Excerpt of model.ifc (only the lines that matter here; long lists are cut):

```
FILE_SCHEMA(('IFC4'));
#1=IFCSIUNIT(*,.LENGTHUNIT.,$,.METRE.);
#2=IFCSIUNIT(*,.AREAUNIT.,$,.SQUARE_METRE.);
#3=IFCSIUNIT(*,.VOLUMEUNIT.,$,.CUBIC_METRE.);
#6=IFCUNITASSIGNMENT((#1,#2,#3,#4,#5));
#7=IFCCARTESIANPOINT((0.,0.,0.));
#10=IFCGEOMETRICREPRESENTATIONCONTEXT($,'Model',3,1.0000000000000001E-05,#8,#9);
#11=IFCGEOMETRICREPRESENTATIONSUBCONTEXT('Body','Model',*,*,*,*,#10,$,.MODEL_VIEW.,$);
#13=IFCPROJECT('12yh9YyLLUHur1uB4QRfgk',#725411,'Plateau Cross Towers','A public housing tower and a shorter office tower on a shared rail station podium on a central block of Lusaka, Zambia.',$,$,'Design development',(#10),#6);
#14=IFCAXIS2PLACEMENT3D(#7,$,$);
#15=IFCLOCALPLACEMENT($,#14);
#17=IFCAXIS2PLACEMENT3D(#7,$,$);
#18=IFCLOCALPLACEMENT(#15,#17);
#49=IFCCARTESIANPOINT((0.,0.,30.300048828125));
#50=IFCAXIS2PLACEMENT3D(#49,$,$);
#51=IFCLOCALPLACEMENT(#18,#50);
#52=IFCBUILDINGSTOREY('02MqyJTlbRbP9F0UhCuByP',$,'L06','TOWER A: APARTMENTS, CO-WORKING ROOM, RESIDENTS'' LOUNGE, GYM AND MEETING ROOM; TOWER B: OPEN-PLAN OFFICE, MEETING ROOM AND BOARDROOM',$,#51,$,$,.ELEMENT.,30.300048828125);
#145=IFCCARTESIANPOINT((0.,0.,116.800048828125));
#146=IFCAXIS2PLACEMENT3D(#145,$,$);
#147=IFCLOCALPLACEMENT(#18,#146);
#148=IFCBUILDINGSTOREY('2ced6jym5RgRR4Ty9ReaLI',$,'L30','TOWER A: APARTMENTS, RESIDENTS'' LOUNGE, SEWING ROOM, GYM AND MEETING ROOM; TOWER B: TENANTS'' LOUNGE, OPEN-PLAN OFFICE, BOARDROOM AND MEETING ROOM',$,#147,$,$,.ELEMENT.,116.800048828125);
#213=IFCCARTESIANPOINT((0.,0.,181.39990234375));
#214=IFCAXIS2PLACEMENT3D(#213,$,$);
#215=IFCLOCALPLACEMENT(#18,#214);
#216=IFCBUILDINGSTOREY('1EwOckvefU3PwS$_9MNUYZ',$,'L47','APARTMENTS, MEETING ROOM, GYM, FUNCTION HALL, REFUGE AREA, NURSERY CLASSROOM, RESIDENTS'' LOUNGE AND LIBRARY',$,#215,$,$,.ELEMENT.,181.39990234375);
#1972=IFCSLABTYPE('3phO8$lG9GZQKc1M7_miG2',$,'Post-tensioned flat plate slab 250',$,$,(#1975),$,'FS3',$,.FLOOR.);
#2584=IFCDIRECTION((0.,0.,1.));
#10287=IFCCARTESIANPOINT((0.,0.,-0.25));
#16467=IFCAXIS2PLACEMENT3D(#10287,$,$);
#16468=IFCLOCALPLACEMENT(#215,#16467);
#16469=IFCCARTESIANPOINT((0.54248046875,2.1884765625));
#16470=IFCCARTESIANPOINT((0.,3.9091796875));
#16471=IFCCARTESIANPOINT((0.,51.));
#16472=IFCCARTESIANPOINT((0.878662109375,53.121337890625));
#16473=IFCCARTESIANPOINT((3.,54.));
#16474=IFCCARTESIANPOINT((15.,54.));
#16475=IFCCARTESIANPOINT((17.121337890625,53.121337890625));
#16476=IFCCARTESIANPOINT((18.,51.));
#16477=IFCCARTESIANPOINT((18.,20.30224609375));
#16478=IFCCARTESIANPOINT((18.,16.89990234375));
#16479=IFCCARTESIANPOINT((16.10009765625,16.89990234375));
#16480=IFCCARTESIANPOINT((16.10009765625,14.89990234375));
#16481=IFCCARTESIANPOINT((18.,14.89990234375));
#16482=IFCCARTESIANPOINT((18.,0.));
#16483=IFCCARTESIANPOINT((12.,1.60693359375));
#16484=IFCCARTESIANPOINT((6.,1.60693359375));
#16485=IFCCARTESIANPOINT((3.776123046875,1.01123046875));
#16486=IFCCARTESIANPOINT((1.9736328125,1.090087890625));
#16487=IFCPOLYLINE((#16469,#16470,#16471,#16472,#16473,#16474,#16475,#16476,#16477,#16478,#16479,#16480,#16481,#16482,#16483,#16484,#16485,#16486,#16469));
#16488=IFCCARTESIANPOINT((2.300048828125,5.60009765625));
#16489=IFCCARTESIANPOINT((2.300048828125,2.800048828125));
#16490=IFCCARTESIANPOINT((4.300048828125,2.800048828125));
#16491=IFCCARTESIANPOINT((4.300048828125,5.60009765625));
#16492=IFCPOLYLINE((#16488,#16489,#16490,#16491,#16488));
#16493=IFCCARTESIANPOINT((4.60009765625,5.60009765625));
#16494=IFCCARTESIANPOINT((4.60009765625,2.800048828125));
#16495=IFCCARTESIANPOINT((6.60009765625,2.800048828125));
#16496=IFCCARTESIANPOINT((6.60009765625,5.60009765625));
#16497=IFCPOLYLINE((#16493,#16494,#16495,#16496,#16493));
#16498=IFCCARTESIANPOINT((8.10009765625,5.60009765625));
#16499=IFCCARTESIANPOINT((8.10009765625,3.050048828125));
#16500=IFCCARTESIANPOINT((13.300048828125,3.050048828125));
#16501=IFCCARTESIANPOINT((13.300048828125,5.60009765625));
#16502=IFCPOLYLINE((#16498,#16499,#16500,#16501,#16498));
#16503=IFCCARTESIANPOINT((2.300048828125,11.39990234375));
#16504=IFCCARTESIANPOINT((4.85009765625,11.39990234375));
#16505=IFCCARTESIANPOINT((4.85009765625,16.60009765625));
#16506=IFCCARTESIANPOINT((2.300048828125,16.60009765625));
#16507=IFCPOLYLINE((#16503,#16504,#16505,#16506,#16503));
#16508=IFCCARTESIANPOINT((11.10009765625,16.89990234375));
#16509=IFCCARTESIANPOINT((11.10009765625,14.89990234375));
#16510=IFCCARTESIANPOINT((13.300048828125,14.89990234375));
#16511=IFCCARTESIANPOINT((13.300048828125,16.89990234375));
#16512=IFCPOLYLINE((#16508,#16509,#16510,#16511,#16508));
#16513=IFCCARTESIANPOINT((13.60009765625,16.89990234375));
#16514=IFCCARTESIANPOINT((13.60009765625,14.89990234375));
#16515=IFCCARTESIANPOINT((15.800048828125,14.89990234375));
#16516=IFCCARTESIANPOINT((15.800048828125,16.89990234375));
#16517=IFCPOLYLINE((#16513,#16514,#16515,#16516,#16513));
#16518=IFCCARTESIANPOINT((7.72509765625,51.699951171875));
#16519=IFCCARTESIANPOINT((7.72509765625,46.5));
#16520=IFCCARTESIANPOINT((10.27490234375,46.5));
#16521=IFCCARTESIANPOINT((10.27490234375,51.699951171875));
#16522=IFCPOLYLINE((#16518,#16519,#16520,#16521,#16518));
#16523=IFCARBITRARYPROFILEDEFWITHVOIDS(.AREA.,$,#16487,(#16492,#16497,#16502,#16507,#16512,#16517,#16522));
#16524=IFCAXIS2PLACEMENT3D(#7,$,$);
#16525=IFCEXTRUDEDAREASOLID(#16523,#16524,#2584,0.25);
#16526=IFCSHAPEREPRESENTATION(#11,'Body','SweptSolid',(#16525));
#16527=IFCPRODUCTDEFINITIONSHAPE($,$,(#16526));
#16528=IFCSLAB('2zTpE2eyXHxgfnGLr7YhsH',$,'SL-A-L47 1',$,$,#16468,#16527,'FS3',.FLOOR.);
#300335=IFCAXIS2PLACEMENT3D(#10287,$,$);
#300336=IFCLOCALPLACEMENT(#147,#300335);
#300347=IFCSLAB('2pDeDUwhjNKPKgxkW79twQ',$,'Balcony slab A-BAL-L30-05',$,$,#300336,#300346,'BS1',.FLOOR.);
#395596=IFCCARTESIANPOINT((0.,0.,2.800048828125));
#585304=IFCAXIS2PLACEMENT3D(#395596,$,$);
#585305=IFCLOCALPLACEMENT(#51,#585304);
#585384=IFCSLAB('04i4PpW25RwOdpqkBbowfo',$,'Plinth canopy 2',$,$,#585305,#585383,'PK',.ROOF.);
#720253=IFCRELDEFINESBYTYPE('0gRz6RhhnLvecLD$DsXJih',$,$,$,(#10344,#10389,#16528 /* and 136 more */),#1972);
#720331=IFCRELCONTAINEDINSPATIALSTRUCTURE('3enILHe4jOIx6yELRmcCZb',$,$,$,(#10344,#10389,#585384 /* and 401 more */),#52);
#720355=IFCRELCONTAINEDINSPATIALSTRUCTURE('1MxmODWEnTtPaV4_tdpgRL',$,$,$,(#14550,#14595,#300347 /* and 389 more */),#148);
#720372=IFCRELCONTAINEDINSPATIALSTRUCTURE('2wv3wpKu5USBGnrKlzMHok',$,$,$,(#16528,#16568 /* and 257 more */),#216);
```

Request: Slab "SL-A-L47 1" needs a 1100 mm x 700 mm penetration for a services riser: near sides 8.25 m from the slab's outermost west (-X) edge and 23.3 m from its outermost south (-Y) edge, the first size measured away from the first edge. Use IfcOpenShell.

```python
import numpy as np
import ifcopenshell
import ifcopenshell.api.feature
import ifcopenshell.api.geometry
import ifcopenshell.api.root
import ifcopenshell.geom
import ifcopenshell.util.placement
import ifcopenshell.util.representation
import ifcopenshell.util.shape
import ifcopenshell.util.unit

model = ifcopenshell.open("model.ifc")
unit_scale = ifcopenshell.util.unit.calculate_unit_scale(model)
settings = ifcopenshell.geom.settings()


def volume(element):
    """Net volume in cubic metres, openings subtracted."""
    shape = ifcopenshell.geom.create_shape(settings, element)
    return ifcopenshell.util.shape.get_volume(shape.geometry)


slab = model.by_guid("2zTpE2eyXHxgfnGLr7YhsH")
before = volume(slab)

# Extent in the slab's own axes, in metres. The edges named are its -X and -Y sides.
slab_shape = ifcopenshell.geom.create_shape(settings, slab)
vertices = ifcopenshell.util.shape.get_vertices(slab_shape.geometry)
x_min, y_min, bottom = vertices.min(axis=0)
top = vertices[:, 2].max()

opening = ifcopenshell.api.root.create_entity(model, ifc_class="IfcOpeningElement", name="Services riser opening", predefined_type="OPENING")
context = ifcopenshell.util.representation.get_context(model, "Model", "Body", "MODEL_VIEW")
width, depth = 1.1, 0.7
outline = [(0.0, 0.0), (width, 0.0), (width, depth), (0.0, depth), (0.0, 0.0)]
# Overshoot both faces by 50 mm so the cut is clean.
shape = ifcopenshell.api.geometry.add_slab_representation(
    model, context=context, depth=top - bottom + 0.1, polyline=outline
)
ifcopenshell.api.geometry.assign_representation(model, product=opening, representation=shape)

matrix = ifcopenshell.util.placement.get_local_placement(slab.ObjectPlacement)
matrix[:, 3] = matrix @ np.append(np.array([x_min + 8.25, y_min + 23.3, bottom - 0.05]) / unit_scale, 1.0)
ifcopenshell.api.geometry.edit_object_placement(model, product=opening, matrix=matrix, is_si=False)
ifcopenshell.api.feature.add_feature(model, feature=opening, element=slab)

after = volume(slab)

print(f"slab volume {before:.3f} -> {after:.3f} m3")

model.write("model_updated.ifc")
```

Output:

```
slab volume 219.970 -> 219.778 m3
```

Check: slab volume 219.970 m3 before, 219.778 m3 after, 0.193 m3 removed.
